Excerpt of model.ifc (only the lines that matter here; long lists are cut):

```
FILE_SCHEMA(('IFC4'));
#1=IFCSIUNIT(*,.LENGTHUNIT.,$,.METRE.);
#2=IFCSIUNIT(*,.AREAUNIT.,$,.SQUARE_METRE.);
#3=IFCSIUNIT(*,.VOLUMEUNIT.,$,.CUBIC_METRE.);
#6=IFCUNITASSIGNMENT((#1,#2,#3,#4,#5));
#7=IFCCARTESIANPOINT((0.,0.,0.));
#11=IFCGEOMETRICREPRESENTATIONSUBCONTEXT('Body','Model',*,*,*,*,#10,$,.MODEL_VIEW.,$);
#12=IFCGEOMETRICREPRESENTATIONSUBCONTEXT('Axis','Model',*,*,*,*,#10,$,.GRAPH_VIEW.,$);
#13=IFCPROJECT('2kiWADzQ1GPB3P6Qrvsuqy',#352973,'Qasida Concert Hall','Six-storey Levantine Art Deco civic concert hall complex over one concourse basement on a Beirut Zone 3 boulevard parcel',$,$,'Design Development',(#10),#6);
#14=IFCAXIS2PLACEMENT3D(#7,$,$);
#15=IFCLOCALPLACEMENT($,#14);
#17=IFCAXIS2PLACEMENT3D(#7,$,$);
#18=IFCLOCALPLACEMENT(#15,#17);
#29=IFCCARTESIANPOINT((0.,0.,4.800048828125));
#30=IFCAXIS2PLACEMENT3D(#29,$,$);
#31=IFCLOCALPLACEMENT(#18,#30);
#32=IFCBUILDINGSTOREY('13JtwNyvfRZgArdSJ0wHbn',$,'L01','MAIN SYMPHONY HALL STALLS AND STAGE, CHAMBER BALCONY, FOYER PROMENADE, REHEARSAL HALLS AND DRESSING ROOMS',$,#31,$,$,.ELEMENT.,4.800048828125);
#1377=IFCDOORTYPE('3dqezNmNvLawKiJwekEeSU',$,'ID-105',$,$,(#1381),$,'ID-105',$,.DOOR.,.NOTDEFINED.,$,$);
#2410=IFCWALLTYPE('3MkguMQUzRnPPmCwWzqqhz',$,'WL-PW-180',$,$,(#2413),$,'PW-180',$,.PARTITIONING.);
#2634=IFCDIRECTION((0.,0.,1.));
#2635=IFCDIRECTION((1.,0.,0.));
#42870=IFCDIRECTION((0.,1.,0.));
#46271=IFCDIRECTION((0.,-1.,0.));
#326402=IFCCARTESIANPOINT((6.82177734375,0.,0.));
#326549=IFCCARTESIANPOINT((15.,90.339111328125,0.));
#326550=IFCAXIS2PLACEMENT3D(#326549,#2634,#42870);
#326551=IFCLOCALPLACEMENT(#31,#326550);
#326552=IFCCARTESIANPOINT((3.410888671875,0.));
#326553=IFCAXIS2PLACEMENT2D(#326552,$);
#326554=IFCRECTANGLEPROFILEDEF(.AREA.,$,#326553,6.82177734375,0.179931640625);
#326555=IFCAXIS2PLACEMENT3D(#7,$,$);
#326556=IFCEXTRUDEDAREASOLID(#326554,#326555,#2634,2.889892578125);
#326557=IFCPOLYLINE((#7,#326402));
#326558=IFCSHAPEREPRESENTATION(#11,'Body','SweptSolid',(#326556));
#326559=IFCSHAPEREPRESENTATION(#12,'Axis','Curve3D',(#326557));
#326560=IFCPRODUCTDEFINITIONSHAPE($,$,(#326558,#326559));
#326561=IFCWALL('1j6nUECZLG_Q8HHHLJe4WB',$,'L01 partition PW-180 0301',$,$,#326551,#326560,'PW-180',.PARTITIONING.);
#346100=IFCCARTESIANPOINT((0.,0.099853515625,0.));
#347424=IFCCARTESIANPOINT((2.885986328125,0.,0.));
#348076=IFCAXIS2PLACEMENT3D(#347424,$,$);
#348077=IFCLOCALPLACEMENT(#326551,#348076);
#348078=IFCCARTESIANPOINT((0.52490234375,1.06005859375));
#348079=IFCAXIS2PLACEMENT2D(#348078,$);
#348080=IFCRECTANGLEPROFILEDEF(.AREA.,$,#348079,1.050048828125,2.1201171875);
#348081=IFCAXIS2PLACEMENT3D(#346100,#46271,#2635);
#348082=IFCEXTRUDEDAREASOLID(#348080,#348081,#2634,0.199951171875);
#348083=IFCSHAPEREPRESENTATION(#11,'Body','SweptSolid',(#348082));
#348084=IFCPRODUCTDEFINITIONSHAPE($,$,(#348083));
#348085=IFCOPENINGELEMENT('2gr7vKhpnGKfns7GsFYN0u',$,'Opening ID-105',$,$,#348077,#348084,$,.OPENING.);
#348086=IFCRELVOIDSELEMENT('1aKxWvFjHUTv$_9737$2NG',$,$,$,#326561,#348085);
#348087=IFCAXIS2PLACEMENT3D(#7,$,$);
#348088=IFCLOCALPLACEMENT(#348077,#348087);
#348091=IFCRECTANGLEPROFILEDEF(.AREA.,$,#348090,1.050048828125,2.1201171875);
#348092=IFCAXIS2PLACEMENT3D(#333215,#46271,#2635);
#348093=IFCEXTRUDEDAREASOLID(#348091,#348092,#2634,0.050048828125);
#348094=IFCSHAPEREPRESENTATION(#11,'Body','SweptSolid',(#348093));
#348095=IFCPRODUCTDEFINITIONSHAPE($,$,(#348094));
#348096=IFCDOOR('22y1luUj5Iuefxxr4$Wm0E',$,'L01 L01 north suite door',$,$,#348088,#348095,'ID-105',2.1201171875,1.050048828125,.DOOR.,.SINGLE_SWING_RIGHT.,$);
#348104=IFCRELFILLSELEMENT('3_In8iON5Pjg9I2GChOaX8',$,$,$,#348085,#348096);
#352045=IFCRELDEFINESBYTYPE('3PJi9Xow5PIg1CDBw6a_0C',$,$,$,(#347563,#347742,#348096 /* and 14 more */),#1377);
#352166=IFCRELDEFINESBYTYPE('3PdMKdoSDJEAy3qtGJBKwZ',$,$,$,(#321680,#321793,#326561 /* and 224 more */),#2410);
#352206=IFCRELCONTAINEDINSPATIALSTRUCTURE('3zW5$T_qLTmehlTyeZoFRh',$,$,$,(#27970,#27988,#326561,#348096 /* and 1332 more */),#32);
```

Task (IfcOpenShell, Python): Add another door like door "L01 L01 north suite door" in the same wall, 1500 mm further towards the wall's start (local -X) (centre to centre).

```python
import ifcopenshell
import ifcopenshell.api.feature
import ifcopenshell.api.geometry
import ifcopenshell.api.root
import ifcopenshell.geom
import ifcopenshell.util.element
import ifcopenshell.util.placement
import ifcopenshell.util.shape
import ifcopenshell.util.unit

model = ifcopenshell.open("model.ifc")
unit_scale = ifcopenshell.util.unit.calculate_unit_scale(model)
settings = ifcopenshell.geom.settings()


def volume(element):
    """Net volume in cubic metres, openings subtracted."""
    shape = ifcopenshell.geom.create_shape(settings, element)
    return ifcopenshell.util.shape.get_volume(shape.geometry)


door = model.by_guid("22y1luUj5Iuefxxr4$Wm0E")
opening = door.FillsVoids[0].RelatingOpeningElement
wall = opening.VoidsElements[0].RelatingBuildingElement
before = volume(wall)
shift = ifcopenshell.util.placement.get_local_placement(wall.ObjectPlacement)[:3, 0] * -1.5 / unit_scale

# copy_class copies the void relationship, type, container and properties, but no geometry.
new_opening = ifcopenshell.api.root.copy_class(model, product=opening)
new_opening.Representation = ifcopenshell.util.element.copy_deep(
    model, opening.Representation, exclude=["IfcGeometricRepresentationContext", "IfcRepresentationMap"]
)
new_door = ifcopenshell.api.root.copy_class(model, product=door)
new_door.Representation = ifcopenshell.util.element.copy_deep(
    model, door.Representation, exclude=["IfcGeometricRepresentationContext", "IfcRepresentationMap"]
)
new_door.Tag = None
ifcopenshell.api.feature.add_filling(model, opening=new_opening, element=new_door)

for old, new in ((opening, new_opening), (door, new_door)):
    matrix = ifcopenshell.util.placement.get_local_placement(old.ObjectPlacement)
    matrix[:3, 3] += shift
    ifcopenshell.api.geometry.edit_object_placement(model, product=new, matrix=matrix, is_si=False)

after = volume(wall)

print(f"wall volume {before:.3f} -> {after:.3f} m3")

model.write("model_v2.ifc")
```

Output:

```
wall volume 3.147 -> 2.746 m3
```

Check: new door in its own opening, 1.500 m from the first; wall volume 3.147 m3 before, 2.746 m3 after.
